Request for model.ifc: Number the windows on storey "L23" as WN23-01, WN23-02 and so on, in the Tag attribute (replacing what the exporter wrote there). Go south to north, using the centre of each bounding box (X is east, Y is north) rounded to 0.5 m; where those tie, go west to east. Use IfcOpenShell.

First a look at what the model holds.

```python
import ifcopenshell
import ifcopenshell.util.element
import ifcopenshell.util.placement

model = ifcopenshell.open("model.ifc")
print(model.schema)
storey = next(s for s in model.by_type("IfcBuildingStorey") if s.Name == "L23")
windows = [e for e in ifcopenshell.util.element.get_decomposition(storey) if e.is_a("IfcWindow")]
for e in sorted(windows, key=lambda e: e.id()):
    origin = ifcopenshell.util.placement.get_local_placement(e.ObjectPlacement)[:3, 3]
    print(e.id(), e.Tag, e.Name, origin.round(2) + 0.0, sep=" | ")
```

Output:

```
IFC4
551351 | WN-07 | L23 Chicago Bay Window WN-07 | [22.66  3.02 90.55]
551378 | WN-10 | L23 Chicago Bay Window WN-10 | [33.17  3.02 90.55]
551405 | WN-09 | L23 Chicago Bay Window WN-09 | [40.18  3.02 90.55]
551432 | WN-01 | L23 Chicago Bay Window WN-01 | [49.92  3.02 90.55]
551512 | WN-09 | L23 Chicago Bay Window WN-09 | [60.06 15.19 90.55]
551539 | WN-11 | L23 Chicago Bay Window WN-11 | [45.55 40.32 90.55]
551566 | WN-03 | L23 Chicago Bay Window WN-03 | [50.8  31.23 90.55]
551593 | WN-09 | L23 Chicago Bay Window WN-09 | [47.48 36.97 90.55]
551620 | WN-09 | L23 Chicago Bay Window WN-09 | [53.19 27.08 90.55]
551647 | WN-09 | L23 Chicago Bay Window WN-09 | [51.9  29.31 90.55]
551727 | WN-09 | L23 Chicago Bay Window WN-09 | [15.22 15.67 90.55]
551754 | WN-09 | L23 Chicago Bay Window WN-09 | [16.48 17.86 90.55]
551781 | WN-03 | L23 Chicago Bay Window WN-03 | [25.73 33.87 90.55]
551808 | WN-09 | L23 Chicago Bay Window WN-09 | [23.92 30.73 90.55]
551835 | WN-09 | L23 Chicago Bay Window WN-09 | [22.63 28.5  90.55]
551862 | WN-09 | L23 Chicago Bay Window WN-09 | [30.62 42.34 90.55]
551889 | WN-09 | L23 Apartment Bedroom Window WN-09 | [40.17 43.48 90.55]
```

```python
import ifcopenshell
import ifcopenshell.geom
import ifcopenshell.util.element
import ifcopenshell.util.shape

model = ifcopenshell.open("model.ifc")
settings = ifcopenshell.geom.settings()
settings.set("use-world-coords", True)


def centre(element):
    shape = ifcopenshell.geom.create_shape(settings, element)
    return ifcopenshell.util.shape.get_bbox_centroid(shape.geometry)


storey = next(s for s in model.by_type("IfcBuildingStorey") if s.Name == "L23")
windows = [e for e in ifcopenshell.util.element.get_decomposition(storey) if e.is_a("IfcWindow")]

# Insertion points can sit at a corner or the storey origin, so sort by the geometry (in metres).
centres = {e: centre(e) for e in windows}
windows.sort(key=lambda e: (round(centres[e][1] / 0.5), centres[e][0]))

for i, e in enumerate(windows, start=1):
    number = f"WN23-{i:02d}"
    e.Tag = number
    print(e.id(), number)

model.write("model-out.ifc")
```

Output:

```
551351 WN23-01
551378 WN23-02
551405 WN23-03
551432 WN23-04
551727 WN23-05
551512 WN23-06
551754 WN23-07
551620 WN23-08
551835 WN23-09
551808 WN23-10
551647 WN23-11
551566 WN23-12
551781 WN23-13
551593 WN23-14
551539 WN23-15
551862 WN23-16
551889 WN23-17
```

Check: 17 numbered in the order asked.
